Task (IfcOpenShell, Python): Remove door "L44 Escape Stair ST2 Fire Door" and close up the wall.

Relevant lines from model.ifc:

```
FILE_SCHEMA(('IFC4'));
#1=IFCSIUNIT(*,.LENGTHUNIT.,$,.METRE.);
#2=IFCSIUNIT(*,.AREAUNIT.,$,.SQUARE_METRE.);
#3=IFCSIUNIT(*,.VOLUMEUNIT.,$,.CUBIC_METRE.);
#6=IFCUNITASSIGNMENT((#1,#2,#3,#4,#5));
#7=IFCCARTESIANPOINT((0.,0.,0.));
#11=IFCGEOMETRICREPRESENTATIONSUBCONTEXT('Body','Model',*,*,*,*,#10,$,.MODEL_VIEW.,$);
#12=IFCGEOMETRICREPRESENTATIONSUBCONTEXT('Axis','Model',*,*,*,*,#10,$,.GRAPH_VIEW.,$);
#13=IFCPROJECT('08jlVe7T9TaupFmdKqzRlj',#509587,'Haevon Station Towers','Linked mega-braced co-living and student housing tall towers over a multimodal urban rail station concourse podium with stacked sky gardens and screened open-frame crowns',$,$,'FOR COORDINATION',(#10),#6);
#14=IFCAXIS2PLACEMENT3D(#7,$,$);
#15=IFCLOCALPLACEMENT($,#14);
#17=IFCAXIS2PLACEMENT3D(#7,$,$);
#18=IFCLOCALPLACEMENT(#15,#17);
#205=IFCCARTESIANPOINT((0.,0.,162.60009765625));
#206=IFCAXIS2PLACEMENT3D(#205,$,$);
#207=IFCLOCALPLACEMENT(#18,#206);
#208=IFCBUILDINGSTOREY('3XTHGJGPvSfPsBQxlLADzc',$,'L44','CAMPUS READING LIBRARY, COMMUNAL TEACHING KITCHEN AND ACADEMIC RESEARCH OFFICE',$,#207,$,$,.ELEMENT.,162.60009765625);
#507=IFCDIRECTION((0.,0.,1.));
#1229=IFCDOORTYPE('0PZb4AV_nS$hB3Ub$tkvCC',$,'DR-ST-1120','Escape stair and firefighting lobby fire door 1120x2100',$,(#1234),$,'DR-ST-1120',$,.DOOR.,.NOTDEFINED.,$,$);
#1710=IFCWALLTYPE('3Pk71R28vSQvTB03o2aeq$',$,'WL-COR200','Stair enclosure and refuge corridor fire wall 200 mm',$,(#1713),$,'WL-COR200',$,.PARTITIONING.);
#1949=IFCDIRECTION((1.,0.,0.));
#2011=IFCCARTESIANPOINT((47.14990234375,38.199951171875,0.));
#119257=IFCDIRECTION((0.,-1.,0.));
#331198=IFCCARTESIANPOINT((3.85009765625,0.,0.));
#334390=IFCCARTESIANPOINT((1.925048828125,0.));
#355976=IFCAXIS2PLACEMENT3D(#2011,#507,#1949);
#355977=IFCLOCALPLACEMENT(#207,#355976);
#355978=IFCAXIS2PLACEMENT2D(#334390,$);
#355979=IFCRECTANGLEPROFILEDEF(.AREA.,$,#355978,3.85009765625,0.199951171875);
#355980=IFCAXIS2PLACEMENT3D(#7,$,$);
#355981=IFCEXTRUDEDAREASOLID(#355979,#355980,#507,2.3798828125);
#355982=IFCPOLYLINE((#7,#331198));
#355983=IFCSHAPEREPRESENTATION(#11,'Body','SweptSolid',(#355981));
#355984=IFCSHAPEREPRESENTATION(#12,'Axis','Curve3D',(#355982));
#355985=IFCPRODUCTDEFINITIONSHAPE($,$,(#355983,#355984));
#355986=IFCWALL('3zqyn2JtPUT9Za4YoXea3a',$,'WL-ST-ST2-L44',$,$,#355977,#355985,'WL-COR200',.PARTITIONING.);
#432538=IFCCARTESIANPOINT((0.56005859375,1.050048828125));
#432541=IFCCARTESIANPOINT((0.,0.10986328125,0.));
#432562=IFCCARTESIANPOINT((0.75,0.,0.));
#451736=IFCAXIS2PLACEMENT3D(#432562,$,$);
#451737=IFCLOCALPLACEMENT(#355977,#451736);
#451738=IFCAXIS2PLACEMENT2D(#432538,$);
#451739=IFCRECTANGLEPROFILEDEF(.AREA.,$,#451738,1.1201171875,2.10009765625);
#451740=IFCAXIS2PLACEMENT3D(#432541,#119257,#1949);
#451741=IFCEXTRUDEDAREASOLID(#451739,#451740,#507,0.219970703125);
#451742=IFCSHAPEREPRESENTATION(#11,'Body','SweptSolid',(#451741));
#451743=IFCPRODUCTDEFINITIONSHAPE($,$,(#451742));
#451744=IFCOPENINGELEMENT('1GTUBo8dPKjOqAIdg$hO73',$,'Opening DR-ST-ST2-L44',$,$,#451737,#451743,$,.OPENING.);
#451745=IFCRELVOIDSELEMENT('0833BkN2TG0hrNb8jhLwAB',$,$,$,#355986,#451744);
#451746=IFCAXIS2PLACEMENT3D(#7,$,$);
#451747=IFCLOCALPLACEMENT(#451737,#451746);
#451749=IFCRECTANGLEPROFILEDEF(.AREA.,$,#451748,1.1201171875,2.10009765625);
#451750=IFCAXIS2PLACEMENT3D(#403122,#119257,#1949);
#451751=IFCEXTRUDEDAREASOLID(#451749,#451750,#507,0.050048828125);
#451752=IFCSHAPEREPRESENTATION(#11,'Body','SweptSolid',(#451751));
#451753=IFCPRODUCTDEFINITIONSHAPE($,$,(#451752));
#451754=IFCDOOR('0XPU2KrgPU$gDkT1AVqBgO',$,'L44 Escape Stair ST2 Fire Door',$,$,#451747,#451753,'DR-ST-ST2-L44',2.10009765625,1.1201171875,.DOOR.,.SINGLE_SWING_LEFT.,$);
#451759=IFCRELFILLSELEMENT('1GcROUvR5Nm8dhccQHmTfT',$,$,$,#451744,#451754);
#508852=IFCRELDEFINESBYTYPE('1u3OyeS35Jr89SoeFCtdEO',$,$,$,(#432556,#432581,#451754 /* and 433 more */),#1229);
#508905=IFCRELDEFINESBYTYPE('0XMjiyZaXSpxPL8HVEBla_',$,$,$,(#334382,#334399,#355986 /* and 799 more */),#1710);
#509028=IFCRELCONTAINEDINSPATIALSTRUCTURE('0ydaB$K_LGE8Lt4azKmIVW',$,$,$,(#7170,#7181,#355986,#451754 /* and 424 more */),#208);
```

```python
import ifcopenshell
import ifcopenshell.api.feature
import ifcopenshell.api.root
import ifcopenshell.geom
import ifcopenshell.util.shape

model = ifcopenshell.open("model.ifc")
settings = ifcopenshell.geom.settings()


def volume(element):
    """Net volume in cubic metres, openings subtracted."""
    shape = ifcopenshell.geom.create_shape(settings, element)
    return ifcopenshell.util.shape.get_volume(shape.geometry)


door = model.by_id(451754)
opening = door.FillsVoids[0].RelatingOpeningElement
wall = opening.VoidsElements[0].RelatingBuildingElement
before = volume(wall)

ifcopenshell.api.root.remove_product(model, product=door)
ifcopenshell.api.feature.remove_feature(model, feature=opening)

after = volume(wall)

print(f"wall volume {before:.3f} -> {after:.3f} m3")

model.write("model_rev.ifc")
```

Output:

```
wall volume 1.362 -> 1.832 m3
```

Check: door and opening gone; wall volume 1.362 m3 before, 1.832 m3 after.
